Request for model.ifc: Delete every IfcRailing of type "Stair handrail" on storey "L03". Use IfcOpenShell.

First a look at what the model holds.

```python
import ifcopenshell
import ifcopenshell.util.element

model = ifcopenshell.open("model.ifc")
print(model.schema)
storey = next(s for s in model.by_type("IfcBuildingStorey") if s.Name == "L03")
railings = [e for e in ifcopenshell.util.element.get_decomposition(storey) if e.is_a("IfcRailing")]
seen = {}
for e in railings:
    element_type = ifcopenshell.util.element.get_type(e)
    name = element_type.Name if element_type not in (None, e) else None
    seen[name] = seen.get(name, 0) + 1
for name, count in sorted(seen.items(), key=str):
    print(count, "x", name)
```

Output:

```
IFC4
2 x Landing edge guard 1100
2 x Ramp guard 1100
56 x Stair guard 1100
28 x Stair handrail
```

```python
import ifcopenshell
import ifcopenshell.api.root
import ifcopenshell.util.element

model = ifcopenshell.open("model.ifc")

storey = next(s for s in model.by_type("IfcBuildingStorey") if s.Name == "L03")
railings = [e for e in ifcopenshell.util.element.get_decomposition(storey) if e.is_a("IfcRailing")]
targets = [e for e in railings if (t := ifcopenshell.util.element.get_type(e)) not in (None, e) and t.Name == "Stair handrail"]

for e in targets:
    ifcopenshell.api.root.remove_product(model, product=e)
print(len(targets), "removed")

model.write("model_v2.ifc")
```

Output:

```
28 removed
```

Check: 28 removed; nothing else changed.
